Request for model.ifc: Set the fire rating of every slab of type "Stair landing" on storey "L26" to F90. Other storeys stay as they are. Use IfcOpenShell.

First a look at what the model holds.

```python
import ifcopenshell
import ifcopenshell.util.element

model = ifcopenshell.open("model.ifc")
print(model.schema)
storey = next(s for s in model.by_type("IfcBuildingStorey") if s.Name == "L26")
slabs = [e for e in ifcopenshell.util.element.get_decomposition(storey) if e.is_a("IfcSlab")]
seen = {}
for e in slabs:
    element_type = ifcopenshell.util.element.get_type(e)
    key = (element_type.Name if element_type != e and element_type else None, ifcopenshell.util.element.get_pset(e, "Pset_SlabCommon", "FireRating"))
    seen[key] = seen.get(key, 0) + 1
for (name, value), count in sorted(seen.items(), key=str):
    print(count, "x", name, "|", value)
```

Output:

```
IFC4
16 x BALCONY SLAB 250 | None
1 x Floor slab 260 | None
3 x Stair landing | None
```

```python
import ifcopenshell
import ifcopenshell.api.pset
import ifcopenshell.util.element

model = ifcopenshell.open("model.ifc")

storey = next(s for s in model.by_type("IfcBuildingStorey") if s.Name == "L26")
slabs = [e for e in ifcopenshell.util.element.get_decomposition(storey) if e.is_a("IfcSlab")]

count = 0
for e in slabs:
    element_type = ifcopenshell.util.element.get_type(e)
    if element_type in (None, e) or element_type.Name != "Stair landing":
        continue
    found = ifcopenshell.util.element.get_pset(e, "Pset_SlabCommon", should_inherit=False)
    if found:
        pset = model.by_id(found["id"])
        if len(ifcopenshell.util.element.get_elements_by_pset(pset)) > 1:
            pset = ifcopenshell.api.pset.unshare_pset(model, products=[e], pset=pset)[0]
    else:
        pset = ifcopenshell.api.pset.add_pset(model, product=e, name="Pset_SlabCommon")
    ifcopenshell.api.pset.edit_pset(model, pset=pset, properties={"FireRating": "F90"})
    count += 1

print(count, "slabs updated")

model.write("model-out.ifc")
```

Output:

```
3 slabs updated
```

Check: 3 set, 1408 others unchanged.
